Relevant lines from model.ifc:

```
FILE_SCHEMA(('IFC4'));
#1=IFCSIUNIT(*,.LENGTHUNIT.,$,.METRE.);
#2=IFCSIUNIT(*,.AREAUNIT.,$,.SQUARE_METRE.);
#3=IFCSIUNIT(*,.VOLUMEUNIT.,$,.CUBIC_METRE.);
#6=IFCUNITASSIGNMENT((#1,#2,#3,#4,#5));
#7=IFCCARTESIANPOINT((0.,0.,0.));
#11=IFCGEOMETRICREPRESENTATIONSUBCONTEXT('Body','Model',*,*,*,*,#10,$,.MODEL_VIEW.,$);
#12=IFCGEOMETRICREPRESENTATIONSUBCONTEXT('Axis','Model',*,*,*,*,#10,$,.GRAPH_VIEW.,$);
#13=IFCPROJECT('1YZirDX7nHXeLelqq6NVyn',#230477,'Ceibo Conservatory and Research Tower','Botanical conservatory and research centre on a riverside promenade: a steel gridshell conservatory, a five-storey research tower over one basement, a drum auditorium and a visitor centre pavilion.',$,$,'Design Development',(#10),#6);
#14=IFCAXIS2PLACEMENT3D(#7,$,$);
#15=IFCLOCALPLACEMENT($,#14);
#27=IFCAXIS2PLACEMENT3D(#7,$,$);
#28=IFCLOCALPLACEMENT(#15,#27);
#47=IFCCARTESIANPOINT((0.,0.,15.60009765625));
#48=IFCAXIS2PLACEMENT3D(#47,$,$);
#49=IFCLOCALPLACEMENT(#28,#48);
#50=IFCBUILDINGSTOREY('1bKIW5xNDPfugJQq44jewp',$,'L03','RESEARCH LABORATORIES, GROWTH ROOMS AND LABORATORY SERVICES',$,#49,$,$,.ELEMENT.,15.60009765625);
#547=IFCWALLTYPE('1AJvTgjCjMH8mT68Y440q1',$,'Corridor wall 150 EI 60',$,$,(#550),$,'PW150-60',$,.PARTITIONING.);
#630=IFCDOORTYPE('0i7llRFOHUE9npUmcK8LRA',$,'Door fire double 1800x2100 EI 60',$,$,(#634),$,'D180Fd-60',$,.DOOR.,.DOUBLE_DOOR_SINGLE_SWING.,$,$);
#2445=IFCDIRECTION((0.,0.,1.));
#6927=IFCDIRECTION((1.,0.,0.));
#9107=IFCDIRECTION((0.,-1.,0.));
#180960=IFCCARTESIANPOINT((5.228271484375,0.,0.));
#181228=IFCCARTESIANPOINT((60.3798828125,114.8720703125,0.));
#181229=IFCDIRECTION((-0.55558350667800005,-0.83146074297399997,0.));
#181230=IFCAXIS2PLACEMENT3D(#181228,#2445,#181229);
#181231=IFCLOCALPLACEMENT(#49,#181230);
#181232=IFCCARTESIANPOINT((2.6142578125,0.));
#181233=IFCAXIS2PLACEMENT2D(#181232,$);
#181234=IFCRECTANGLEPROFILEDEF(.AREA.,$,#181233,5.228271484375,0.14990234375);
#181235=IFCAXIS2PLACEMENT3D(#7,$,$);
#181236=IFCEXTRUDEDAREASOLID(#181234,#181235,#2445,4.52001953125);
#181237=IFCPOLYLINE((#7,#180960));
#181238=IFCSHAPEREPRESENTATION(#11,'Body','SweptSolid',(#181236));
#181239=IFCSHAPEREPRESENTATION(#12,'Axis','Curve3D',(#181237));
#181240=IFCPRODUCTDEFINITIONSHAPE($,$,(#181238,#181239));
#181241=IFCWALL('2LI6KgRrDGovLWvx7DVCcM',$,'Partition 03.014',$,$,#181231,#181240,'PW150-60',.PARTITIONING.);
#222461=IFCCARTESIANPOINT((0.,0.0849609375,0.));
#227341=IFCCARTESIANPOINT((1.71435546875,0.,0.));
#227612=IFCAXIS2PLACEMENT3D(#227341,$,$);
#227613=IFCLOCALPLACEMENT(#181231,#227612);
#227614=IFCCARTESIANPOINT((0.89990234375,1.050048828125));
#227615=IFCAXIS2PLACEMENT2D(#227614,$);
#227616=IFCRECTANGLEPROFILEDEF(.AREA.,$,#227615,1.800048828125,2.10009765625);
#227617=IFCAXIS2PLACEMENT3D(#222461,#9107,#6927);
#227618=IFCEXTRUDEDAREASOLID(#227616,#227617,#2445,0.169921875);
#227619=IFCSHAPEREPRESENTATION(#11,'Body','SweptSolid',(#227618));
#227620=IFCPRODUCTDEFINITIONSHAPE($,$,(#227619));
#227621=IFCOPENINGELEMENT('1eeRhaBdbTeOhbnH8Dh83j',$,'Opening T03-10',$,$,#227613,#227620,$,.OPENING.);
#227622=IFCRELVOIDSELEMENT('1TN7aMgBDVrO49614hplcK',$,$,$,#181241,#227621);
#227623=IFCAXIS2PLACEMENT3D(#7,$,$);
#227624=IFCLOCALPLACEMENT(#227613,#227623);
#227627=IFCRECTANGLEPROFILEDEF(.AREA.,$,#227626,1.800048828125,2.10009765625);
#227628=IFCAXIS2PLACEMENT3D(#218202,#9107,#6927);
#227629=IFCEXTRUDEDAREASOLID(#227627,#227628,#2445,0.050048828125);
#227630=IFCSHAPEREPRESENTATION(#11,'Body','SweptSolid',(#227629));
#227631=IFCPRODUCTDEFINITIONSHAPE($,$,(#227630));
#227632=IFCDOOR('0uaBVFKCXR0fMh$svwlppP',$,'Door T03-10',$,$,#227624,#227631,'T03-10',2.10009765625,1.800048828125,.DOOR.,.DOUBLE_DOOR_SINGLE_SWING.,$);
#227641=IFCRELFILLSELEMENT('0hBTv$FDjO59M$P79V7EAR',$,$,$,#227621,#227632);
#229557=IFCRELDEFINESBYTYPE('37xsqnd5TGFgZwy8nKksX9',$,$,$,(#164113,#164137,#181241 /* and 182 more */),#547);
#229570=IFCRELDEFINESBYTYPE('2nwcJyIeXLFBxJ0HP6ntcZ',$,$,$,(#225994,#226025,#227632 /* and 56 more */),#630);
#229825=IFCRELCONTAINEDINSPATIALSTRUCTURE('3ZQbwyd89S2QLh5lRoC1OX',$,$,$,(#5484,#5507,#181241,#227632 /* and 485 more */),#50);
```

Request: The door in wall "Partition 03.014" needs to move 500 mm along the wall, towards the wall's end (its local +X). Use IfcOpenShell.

```python
import ifcopenshell
import ifcopenshell.api.geometry
import ifcopenshell.util.placement
import ifcopenshell.util.unit

model = ifcopenshell.open("model.ifc")
unit_scale = ifcopenshell.util.unit.calculate_unit_scale(model)

door = model.by_id(227632)
opening = door.FillsVoids[0].RelatingOpeningElement
wall = opening.VoidsElements[0].RelatingBuildingElement

wall_matrix = ifcopenshell.util.placement.get_local_placement(wall.ObjectPlacement)
shift = wall_matrix[:3, 0] * 0.5 / unit_scale
before = ifcopenshell.util.placement.get_local_placement(door.ObjectPlacement)[:3, 3].copy()

# The door is placed relative to its opening, so it follows when the opening moves.
matrix = ifcopenshell.util.placement.get_local_placement(opening.ObjectPlacement)
matrix[:3, 3] += shift
ifcopenshell.api.geometry.edit_object_placement(
    model, product=opening, matrix=matrix, is_si=False, should_transform_children=True
)

after = ifcopenshell.util.placement.get_local_placement(door.ObjectPlacement)[:3, 3]
print("door moved by", (after - before).round(3) + 0.0)

model.write("model_rev.ifc")
```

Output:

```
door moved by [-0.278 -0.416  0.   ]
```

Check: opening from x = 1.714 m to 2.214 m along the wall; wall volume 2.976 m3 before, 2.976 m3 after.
